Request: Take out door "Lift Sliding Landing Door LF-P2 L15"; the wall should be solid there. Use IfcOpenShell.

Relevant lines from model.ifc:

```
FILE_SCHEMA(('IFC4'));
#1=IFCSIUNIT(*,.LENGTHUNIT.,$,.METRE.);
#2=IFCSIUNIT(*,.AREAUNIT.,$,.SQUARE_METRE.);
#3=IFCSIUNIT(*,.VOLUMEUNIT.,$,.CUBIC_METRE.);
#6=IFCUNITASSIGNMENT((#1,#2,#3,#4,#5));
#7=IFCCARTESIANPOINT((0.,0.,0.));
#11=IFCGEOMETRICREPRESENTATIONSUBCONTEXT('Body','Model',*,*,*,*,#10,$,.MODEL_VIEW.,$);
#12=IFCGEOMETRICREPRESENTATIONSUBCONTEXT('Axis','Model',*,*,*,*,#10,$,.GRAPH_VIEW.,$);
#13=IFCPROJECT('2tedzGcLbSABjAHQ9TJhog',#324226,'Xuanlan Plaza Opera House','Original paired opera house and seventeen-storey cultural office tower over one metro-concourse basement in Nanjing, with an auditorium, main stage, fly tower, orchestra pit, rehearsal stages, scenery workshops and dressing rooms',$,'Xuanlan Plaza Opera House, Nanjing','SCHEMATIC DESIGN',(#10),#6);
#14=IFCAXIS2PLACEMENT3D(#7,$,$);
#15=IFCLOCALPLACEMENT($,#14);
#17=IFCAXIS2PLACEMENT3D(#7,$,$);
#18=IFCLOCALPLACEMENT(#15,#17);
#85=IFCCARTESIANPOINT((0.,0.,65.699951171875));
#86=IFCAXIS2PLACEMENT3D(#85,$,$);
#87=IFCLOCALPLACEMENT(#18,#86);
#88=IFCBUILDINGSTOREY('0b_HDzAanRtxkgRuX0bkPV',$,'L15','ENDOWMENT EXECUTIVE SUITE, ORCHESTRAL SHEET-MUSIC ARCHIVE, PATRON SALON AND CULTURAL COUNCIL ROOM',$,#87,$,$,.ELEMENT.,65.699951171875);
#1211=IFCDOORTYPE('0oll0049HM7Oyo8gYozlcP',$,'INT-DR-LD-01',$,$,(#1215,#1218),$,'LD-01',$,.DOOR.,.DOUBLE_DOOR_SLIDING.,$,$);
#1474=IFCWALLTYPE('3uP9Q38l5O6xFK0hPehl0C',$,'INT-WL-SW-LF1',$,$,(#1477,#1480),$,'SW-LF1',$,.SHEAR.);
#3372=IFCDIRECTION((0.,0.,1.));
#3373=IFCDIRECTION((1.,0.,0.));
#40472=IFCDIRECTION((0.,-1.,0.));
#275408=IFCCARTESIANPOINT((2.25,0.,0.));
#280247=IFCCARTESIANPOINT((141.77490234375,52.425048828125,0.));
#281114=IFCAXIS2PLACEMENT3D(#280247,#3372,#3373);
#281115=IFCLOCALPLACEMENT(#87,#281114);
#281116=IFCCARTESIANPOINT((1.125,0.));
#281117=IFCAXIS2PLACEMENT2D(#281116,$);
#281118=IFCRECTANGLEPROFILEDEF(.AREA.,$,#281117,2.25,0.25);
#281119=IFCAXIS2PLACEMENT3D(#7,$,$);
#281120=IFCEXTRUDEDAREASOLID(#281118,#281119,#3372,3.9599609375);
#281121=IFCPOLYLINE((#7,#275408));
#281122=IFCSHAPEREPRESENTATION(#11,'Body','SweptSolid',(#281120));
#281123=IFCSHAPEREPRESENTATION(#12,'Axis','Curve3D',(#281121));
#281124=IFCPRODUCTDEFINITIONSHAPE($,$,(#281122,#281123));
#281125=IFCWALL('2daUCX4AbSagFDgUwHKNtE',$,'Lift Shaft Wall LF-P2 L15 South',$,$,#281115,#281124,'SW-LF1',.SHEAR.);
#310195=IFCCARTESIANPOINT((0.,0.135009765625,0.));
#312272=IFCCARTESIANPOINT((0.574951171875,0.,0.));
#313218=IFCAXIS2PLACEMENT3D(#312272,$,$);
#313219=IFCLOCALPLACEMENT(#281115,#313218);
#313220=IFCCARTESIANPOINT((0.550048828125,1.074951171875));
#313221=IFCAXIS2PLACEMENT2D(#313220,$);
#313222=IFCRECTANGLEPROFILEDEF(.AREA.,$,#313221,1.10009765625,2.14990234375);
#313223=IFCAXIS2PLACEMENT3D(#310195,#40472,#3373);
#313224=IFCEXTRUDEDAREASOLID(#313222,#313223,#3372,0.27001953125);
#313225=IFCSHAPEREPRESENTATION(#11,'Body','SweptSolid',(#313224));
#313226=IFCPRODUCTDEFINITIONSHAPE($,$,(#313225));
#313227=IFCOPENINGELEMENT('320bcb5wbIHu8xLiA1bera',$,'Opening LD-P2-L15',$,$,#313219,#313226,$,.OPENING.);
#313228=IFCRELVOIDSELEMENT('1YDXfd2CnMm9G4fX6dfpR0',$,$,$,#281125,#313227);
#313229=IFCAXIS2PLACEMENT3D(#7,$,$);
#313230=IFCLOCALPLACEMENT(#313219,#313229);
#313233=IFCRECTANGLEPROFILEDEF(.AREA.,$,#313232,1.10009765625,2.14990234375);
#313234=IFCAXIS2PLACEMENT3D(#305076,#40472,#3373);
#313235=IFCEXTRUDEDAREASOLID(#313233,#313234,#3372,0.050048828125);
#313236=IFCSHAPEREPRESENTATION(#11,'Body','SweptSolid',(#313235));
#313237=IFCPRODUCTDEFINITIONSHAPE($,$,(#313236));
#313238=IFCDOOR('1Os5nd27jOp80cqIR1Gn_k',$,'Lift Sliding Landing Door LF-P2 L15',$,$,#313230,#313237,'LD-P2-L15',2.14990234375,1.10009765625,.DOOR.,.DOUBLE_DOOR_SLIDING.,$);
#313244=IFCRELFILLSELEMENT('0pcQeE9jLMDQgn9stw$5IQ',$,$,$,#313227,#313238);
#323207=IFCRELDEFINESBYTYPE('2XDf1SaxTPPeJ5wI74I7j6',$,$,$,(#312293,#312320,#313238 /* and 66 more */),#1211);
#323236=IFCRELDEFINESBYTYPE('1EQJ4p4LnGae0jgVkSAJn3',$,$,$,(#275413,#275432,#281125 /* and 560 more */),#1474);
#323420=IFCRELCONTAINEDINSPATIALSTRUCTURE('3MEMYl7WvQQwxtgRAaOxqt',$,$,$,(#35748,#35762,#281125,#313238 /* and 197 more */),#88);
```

```python
import ifcopenshell
import ifcopenshell.api.feature
import ifcopenshell.api.root
import ifcopenshell.geom
import ifcopenshell.util.shape

model = ifcopenshell.open("model.ifc")
settings = ifcopenshell.geom.settings()


def volume(element):
    """Net volume in cubic metres, openings subtracted."""
    shape = ifcopenshell.geom.create_shape(settings, element)
    return ifcopenshell.util.shape.get_volume(shape.geometry)


door = model.by_guid("1Os5nd27jOp80cqIR1Gn_k")
opening = door.FillsVoids[0].RelatingOpeningElement
wall = opening.VoidsElements[0].RelatingBuildingElement
before = volume(wall)

ifcopenshell.api.root.remove_product(model, product=door)
ifcopenshell.api.feature.remove_feature(model, feature=opening)

after = volume(wall)

print(f"wall volume {before:.3f} -> {after:.3f} m3")

model.write("model_v2.ifc")
```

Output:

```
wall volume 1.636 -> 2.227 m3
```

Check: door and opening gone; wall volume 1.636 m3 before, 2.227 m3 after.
